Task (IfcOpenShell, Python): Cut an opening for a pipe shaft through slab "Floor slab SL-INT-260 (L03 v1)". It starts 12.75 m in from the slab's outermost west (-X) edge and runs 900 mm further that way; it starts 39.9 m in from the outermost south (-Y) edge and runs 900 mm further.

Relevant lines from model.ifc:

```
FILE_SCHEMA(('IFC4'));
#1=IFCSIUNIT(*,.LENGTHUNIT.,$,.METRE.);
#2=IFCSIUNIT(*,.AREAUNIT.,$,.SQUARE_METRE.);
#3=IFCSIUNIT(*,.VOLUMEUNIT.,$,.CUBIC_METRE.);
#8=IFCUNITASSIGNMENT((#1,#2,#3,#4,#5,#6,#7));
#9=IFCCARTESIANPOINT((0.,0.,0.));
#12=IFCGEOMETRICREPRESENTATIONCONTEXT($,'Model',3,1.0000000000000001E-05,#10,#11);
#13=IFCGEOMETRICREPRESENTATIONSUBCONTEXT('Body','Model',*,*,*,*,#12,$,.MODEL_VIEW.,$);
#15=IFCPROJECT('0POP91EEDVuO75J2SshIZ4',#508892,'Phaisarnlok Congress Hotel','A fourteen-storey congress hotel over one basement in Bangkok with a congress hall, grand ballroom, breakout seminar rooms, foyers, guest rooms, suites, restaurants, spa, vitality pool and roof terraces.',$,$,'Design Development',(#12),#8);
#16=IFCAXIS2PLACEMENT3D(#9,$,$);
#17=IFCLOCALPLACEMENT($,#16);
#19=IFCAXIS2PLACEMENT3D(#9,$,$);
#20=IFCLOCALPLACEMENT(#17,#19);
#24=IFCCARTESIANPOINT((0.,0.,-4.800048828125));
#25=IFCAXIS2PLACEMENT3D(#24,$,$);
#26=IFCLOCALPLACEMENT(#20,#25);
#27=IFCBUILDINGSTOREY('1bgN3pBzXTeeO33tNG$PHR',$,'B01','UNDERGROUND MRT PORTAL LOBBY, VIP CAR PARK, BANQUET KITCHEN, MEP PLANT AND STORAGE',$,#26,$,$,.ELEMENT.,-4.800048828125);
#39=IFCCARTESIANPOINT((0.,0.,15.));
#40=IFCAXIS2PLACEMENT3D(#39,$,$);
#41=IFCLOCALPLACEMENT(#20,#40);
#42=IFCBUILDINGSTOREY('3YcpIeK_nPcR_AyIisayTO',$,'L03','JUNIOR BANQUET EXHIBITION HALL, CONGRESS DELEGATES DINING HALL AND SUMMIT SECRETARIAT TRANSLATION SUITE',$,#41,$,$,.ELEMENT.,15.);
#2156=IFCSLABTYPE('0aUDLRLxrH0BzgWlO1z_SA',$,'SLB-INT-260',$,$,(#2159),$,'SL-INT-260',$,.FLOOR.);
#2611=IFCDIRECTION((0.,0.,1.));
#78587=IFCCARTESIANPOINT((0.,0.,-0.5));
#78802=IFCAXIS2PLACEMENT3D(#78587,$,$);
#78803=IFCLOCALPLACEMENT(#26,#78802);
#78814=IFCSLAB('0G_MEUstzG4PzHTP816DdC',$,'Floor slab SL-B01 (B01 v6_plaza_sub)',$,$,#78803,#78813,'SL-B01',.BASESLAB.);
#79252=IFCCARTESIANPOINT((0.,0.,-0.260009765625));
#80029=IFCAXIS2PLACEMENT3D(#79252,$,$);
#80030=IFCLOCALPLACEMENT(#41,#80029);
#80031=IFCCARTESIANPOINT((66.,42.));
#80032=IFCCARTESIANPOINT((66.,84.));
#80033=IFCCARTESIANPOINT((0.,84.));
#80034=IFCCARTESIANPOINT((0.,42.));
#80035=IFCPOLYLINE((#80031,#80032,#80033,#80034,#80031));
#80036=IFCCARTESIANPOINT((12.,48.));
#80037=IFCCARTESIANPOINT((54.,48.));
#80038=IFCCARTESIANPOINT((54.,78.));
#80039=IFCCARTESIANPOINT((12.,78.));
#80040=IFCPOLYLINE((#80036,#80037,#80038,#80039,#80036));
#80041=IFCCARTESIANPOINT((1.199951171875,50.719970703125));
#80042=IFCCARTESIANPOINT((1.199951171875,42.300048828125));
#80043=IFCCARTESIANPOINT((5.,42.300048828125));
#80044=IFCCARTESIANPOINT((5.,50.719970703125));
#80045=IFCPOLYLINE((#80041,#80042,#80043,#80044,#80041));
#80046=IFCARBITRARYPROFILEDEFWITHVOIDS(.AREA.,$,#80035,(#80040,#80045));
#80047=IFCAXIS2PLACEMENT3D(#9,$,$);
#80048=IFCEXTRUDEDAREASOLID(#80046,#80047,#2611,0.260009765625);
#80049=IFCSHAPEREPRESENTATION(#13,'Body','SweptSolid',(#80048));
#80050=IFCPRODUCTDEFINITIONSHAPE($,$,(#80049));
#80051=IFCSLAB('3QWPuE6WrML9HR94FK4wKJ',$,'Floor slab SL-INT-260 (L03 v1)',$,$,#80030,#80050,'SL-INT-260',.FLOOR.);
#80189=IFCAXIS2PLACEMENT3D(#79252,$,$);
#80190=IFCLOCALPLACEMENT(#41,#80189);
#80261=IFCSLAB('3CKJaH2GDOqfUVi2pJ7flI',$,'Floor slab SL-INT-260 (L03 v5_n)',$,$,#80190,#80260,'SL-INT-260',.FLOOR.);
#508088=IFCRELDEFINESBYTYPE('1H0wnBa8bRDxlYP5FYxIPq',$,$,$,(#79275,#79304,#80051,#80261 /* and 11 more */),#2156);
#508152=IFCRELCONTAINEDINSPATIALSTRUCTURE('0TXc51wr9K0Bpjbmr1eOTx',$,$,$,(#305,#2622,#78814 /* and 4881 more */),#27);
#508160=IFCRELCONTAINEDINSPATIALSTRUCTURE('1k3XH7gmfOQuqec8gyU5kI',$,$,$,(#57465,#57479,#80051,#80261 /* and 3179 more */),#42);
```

```python
import numpy as np
import ifcopenshell
import ifcopenshell.api.feature
import ifcopenshell.api.geometry
import ifcopenshell.api.root
import ifcopenshell.geom
import ifcopenshell.util.placement
import ifcopenshell.util.representation
import ifcopenshell.util.shape
import ifcopenshell.util.unit

model = ifcopenshell.open("model.ifc")
unit_scale = ifcopenshell.util.unit.calculate_unit_scale(model)
settings = ifcopenshell.geom.settings()


def volume(element):
    """Net volume in cubic metres, openings subtracted."""
    shape = ifcopenshell.geom.create_shape(settings, element)
    return ifcopenshell.util.shape.get_volume(shape.geometry)


slab = model.by_guid("3QWPuE6WrML9HR94FK4wKJ")
before = volume(slab)

# Extent in the slab's own axes, in metres. The edges named are its -X and -Y sides.
slab_shape = ifcopenshell.geom.create_shape(settings, slab)
vertices = ifcopenshell.util.shape.get_vertices(slab_shape.geometry)
x_min, y_min, bottom = vertices.min(axis=0)
top = vertices[:, 2].max()

opening = ifcopenshell.api.root.create_entity(model, ifc_class="IfcOpeningElement", name="Pipe shaft opening", predefined_type="OPENING")
context = ifcopenshell.util.representation.get_context(model, "Model", "Body", "MODEL_VIEW")
width, depth = 0.9, 0.9
outline = [(0.0, 0.0), (width, 0.0), (width, depth), (0.0, depth), (0.0, 0.0)]
# Overshoot both faces by 50 mm so the cut is clean.
shape = ifcopenshell.api.geometry.add_slab_representation(
    model, context=context, depth=top - bottom + 0.1, polyline=outline
)
ifcopenshell.api.geometry.assign_representation(model, product=opening, representation=shape)

matrix = ifcopenshell.util.placement.get_local_placement(slab.ObjectPlacement)
matrix[:, 3] = matrix @ np.append(np.array([x_min + 12.75, y_min + 39.9, bottom - 0.05]) / unit_scale, 1.0)
ifcopenshell.api.geometry.edit_object_placement(model, product=opening, matrix=matrix, is_si=False)
ifcopenshell.api.feature.add_feature(model, feature=opening, element=slab)

after = volume(slab)

print(f"slab volume {before:.3f} -> {after:.3f} m3")

model.write("model_updated.ifc")
```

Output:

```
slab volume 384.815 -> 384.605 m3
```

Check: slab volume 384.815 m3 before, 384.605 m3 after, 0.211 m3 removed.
